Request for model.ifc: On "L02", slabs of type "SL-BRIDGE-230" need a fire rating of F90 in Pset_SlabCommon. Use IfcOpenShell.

First a look at what the model holds.

```python
import ifcopenshell
import ifcopenshell.util.element

model = ifcopenshell.open("model.ifc")
print(model.schema)
storey = next(s for s in model.by_type("IfcBuildingStorey") if s.Name == "L02")
slabs = [e for e in ifcopenshell.util.element.get_decomposition(storey) if e.is_a("IfcSlab")]
seen = {}
for e in slabs:
    element_type = ifcopenshell.util.element.get_type(e)
    key = (element_type.Name if element_type != e and element_type else None, ifcopenshell.util.element.get_pset(e, "Pset_SlabCommon", "FireRating"))
    seen[key] = seen.get(key, 0) + 1
for (name, value), count in sorted(seen.items(), key=str):
    print(count, "x", name, "|", value)
```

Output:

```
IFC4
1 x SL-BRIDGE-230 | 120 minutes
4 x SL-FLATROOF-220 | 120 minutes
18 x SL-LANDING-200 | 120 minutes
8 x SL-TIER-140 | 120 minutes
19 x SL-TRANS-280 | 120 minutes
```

```python
import ifcopenshell
import ifcopenshell.api.pset
import ifcopenshell.util.element

model = ifcopenshell.open("model.ifc")

storey = next(s for s in model.by_type("IfcBuildingStorey") if s.Name == "L02")
slabs = [e for e in ifcopenshell.util.element.get_decomposition(storey) if e.is_a("IfcSlab")]

count = 0
for e in slabs:
    element_type = ifcopenshell.util.element.get_type(e)
    if element_type in (None, e) or element_type.Name != "SL-BRIDGE-230":
        continue
    # add_pset returns the element's existing set when there is one.
    pset = ifcopenshell.api.pset.add_pset(model, product=e, name="Pset_SlabCommon")
    ifcopenshell.api.pset.edit_pset(model, pset=pset, properties={"FireRating": "F90"})
    count += 1

print(count, "slabs updated")

model.write("model_rev.ifc")
```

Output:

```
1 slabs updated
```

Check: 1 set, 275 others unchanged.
